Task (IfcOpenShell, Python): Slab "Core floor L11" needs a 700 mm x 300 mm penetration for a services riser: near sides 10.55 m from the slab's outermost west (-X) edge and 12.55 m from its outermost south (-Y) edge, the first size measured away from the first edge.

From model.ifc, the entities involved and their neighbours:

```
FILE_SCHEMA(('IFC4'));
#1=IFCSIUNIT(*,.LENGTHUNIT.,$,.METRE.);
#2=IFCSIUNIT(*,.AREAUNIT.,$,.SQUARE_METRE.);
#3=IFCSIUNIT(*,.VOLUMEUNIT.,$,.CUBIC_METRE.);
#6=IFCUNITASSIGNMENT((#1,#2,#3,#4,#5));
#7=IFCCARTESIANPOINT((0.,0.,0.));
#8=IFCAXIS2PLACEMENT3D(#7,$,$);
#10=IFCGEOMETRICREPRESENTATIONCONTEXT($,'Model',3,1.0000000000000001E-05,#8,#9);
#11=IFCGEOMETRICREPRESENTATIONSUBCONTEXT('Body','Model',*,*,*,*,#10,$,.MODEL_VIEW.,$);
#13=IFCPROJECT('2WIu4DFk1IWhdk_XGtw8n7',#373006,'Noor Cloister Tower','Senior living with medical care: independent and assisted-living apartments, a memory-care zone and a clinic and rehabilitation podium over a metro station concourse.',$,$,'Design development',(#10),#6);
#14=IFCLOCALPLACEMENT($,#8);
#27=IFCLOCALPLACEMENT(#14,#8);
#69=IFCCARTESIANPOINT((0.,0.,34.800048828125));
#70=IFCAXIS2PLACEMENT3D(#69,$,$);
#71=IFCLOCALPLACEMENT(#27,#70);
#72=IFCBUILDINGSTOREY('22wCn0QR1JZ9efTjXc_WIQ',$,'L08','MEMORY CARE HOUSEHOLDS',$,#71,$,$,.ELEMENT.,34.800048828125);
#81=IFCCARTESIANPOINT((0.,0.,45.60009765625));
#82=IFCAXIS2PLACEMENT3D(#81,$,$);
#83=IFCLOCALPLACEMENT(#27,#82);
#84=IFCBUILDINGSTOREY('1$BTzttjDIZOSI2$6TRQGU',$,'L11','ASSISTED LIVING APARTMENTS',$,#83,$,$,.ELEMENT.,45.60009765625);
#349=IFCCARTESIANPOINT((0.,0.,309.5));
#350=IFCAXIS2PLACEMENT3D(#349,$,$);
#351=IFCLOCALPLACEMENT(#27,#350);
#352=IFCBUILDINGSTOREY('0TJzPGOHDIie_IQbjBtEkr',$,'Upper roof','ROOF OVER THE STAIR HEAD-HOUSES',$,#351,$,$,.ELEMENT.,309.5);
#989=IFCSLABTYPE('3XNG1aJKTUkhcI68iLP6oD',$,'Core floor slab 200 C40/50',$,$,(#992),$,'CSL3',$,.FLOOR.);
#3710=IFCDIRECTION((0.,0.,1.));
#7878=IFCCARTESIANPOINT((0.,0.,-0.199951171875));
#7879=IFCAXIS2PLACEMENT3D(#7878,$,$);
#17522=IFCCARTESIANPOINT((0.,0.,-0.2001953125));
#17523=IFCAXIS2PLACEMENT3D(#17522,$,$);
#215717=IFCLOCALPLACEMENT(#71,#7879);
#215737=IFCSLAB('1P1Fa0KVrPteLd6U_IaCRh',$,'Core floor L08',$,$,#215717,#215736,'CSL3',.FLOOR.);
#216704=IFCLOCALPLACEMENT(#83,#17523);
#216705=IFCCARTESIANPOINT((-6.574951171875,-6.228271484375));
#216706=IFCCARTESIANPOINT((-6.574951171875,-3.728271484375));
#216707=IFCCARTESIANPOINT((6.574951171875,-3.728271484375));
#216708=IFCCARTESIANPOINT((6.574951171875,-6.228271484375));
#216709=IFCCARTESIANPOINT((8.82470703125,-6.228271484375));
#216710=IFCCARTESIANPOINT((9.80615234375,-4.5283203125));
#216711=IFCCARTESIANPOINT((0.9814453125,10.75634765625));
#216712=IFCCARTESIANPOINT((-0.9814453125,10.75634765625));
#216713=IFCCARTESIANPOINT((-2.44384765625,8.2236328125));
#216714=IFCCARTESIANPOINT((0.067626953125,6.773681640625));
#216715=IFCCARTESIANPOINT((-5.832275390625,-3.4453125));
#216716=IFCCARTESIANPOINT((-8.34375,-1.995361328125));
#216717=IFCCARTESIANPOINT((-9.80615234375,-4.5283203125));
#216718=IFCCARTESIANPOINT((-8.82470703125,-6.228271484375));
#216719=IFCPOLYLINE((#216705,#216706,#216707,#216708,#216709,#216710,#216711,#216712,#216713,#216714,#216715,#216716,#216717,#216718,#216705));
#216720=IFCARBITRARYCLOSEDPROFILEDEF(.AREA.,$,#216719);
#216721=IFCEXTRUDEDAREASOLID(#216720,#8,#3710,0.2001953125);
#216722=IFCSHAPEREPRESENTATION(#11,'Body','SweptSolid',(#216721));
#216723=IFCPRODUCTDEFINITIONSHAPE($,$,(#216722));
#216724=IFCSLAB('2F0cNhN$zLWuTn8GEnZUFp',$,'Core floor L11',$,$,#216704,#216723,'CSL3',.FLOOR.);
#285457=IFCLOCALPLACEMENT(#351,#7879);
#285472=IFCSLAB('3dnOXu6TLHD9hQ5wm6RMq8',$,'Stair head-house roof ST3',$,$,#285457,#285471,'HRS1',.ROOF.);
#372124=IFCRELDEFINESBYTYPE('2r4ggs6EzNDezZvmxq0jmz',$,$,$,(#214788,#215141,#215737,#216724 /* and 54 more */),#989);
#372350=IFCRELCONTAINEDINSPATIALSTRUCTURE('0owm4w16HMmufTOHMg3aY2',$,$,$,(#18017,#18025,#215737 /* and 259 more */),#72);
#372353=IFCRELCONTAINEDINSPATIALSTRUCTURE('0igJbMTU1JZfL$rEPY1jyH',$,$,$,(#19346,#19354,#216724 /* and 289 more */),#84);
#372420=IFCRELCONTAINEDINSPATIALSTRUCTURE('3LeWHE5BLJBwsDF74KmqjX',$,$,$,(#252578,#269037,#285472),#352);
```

```python
import numpy as np
import ifcopenshell
import ifcopenshell.api.feature
import ifcopenshell.api.geometry
import ifcopenshell.api.root
import ifcopenshell.geom
import ifcopenshell.util.placement
import ifcopenshell.util.representation
import ifcopenshell.util.shape
import ifcopenshell.util.unit

model = ifcopenshell.open("model.ifc")
unit_scale = ifcopenshell.util.unit.calculate_unit_scale(model)
settings = ifcopenshell.geom.settings()


def volume(element):
    """Net volume in cubic metres, openings subtracted."""
    shape = ifcopenshell.geom.create_shape(settings, element)
    return ifcopenshell.util.shape.get_volume(shape.geometry)


slab = model.by_guid("2F0cNhN$zLWuTn8GEnZUFp")
before = volume(slab)

# Extent in the slab's own axes, in metres. The edges named are its -X and -Y sides.
slab_shape = ifcopenshell.geom.create_shape(settings, slab)
vertices = ifcopenshell.util.shape.get_vertices(slab_shape.geometry)
x_min, y_min, bottom = vertices.min(axis=0)
top = vertices[:, 2].max()

opening = ifcopenshell.api.root.create_entity(model, ifc_class="IfcOpeningElement", name="Services riser opening", predefined_type="OPENING")
context = ifcopenshell.util.representation.get_context(model, "Model", "Body", "MODEL_VIEW")
width, depth = 0.7, 0.3
outline = [(0.0, 0.0), (width, 0.0), (width, depth), (0.0, depth), (0.0, 0.0)]
# Overshoot both faces by 50 mm so the cut is clean.
shape = ifcopenshell.api.geometry.add_slab_representation(
    model, context=context, depth=top - bottom + 0.1, polyline=outline
)
ifcopenshell.api.geometry.assign_representation(model, product=opening, representation=shape)

matrix = ifcopenshell.util.placement.get_local_placement(slab.ObjectPlacement)
matrix[:, 3] = matrix @ np.append(np.array([x_min + 10.55, y_min + 12.55, bottom - 0.05]) / unit_scale, 1.0)
ifcopenshell.api.geometry.edit_object_placement(model, product=opening, matrix=matrix, is_si=False)
ifcopenshell.api.feature.add_feature(model, feature=opening, element=slab)

after = volume(slab)

print(f"slab volume {before:.3f} -> {after:.3f} m3")

model.write("model-out.ifc")
```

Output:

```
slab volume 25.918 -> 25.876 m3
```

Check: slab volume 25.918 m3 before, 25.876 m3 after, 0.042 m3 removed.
